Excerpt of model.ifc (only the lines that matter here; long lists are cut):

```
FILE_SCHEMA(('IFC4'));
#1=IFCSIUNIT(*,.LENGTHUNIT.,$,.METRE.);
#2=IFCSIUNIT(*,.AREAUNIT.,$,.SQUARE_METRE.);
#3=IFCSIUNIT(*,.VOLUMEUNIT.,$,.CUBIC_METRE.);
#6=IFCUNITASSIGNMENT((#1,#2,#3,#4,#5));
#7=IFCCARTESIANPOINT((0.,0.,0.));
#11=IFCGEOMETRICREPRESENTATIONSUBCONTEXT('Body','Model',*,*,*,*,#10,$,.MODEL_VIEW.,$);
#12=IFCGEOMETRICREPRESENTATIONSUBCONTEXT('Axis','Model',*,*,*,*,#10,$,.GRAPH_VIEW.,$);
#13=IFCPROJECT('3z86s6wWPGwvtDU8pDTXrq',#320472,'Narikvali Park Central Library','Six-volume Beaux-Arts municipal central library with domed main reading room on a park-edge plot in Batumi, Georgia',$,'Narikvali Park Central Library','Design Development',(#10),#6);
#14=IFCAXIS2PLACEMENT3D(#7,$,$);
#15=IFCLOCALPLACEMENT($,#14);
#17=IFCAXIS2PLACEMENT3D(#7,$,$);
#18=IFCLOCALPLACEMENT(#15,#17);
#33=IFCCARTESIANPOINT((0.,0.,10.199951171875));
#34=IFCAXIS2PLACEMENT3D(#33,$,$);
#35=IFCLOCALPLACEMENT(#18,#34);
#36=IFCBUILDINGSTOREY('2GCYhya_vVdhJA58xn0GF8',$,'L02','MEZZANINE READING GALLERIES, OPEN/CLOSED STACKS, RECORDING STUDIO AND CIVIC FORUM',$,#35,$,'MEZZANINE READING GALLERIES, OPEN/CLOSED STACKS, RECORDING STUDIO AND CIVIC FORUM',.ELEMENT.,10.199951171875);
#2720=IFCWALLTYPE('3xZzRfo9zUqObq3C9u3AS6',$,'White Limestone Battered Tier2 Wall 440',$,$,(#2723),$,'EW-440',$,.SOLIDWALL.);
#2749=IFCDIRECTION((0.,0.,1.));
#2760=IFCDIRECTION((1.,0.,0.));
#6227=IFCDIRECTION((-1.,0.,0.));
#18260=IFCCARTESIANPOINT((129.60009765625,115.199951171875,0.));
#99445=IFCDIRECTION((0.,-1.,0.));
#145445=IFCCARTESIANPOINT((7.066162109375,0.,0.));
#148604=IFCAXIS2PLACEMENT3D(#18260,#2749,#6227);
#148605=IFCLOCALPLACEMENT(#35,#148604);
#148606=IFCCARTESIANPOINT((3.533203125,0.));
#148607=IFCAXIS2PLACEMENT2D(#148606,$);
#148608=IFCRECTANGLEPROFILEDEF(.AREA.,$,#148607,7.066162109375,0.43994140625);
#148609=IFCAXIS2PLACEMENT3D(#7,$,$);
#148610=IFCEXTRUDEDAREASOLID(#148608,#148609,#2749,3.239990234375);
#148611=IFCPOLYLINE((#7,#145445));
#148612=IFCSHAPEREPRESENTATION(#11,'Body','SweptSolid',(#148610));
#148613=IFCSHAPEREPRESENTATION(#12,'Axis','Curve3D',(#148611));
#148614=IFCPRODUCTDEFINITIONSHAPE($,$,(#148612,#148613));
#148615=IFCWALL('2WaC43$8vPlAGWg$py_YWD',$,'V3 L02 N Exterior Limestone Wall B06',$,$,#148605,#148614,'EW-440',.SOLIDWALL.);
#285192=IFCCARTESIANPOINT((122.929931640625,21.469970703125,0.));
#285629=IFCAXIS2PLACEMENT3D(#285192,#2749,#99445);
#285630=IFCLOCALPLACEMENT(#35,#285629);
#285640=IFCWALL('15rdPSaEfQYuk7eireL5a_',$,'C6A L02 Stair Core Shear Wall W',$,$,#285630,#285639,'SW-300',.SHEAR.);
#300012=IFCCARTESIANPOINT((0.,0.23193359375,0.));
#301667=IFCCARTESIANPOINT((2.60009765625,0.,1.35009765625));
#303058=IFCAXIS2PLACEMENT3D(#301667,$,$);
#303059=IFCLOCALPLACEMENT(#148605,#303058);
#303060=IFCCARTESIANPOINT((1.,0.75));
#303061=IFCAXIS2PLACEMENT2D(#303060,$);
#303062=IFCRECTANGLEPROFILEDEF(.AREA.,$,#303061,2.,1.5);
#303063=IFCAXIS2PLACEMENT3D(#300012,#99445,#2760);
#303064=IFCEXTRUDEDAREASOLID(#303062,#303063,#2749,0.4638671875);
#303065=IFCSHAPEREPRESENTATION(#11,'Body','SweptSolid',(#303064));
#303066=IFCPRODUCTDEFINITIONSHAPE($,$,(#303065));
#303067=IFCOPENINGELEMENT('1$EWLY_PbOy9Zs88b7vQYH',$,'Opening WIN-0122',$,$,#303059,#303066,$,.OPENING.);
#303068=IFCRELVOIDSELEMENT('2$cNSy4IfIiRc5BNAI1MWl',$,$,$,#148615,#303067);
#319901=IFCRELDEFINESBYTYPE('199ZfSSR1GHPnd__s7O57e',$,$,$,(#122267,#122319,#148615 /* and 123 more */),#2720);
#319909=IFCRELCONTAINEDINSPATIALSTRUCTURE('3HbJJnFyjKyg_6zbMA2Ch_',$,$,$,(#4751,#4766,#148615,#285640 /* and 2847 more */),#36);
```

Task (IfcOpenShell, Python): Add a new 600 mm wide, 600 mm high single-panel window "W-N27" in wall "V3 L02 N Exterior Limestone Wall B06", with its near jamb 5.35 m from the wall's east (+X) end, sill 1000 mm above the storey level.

```python
import numpy as np
import ifcopenshell
import ifcopenshell.api.feature
import ifcopenshell.api.geometry
import ifcopenshell.api.root
import ifcopenshell.api.spatial
import ifcopenshell.geom
import ifcopenshell.util.element
import ifcopenshell.util.placement
import ifcopenshell.util.representation
import ifcopenshell.util.shape
import ifcopenshell.util.unit

model = ifcopenshell.open("model.ifc")
unit_scale = ifcopenshell.util.unit.calculate_unit_scale(model)
settings = ifcopenshell.geom.settings()


def volume(element):
    """Net volume in cubic metres, openings subtracted."""
    shape = ifcopenshell.geom.create_shape(settings, element)
    return ifcopenshell.util.shape.get_volume(shape.geometry)


wall = model.by_guid("2WaC43$8vPlAGWg$py_YWD")
storey = ifcopenshell.util.element.get_container(wall, ifc_class="IfcBuildingStorey")
context = ifcopenshell.util.representation.get_context(model, "Model", "Body", "MODEL_VIEW")
before = volume(wall)

width, height, from_end, sill = 0.6, 0.6, 5.35, 1  # metres

# The wall runs along its own X axis, and the end named is its -X end.
wall_shape = ifcopenshell.geom.create_shape(settings, wall)
x, y, z = ifcopenshell.util.shape.get_vertices(wall_shape.geometry).T
start = x.min() + from_end
face, thickness = float(y.min()), float(y.max() - y.min())
wall_matrix = ifcopenshell.util.placement.get_local_placement(wall.ObjectPlacement)
level = ifcopenshell.util.placement.get_local_placement(storey.ObjectPlacement)[2, 3]


def in_wall(x, y):
    """Placement at x, y metres in the wall's axes, at sill height."""
    matrix = wall_matrix.copy()
    matrix[:, 3] = wall_matrix @ np.array([x / unit_scale, y / unit_scale, 0.0, 1.0])
    matrix[2, 3] = level + sill / unit_scale
    return matrix


# Opening: a box that overshoots both wall faces by 50 mm.
opening = ifcopenshell.api.root.create_entity(model, ifc_class="IfcOpeningElement", predefined_type="OPENING")
box = ifcopenshell.api.geometry.add_wall_representation(
    model, context=context, length=width, height=height, thickness=thickness + 0.1
)
ifcopenshell.api.geometry.assign_representation(model, product=opening, representation=box)
ifcopenshell.api.geometry.edit_object_placement(model, product=opening, matrix=in_wall(start, face - 0.05), is_si=False)
ifcopenshell.api.feature.add_feature(model, feature=opening, element=wall)

window = ifcopenshell.api.root.create_entity(model, ifc_class="IfcWindow", name="W-N27", predefined_type="WINDOW")
window.OverallWidth, window.OverallHeight = width / unit_scale, height / unit_scale
window.PartitioningType = "SINGLE_PANEL"
body = ifcopenshell.api.geometry.add_window_representation(
    model,
    context=context,
    overall_width=window.OverallWidth,
    overall_height=window.OverallHeight,
    partition_type="SINGLE_PANEL",
)
ifcopenshell.api.geometry.assign_representation(model, product=window, representation=body)
ifcopenshell.api.spatial.assign_container(model, products=[window], relating_structure=storey)
ifcopenshell.api.feature.add_filling(model, opening=opening, element=window)

# Centre the window in the wall's thickness.
ifcopenshell.api.geometry.edit_object_placement(model, product=window, matrix=in_wall(start, face), is_si=False)
window_shape = ifcopenshell.geom.create_shape(settings, window)
depth = ifcopenshell.util.shape.get_vertices(window_shape.geometry)[:, 1]
offset = face + thickness / 2 - (depth.min() + depth.max()) / 2
ifcopenshell.api.geometry.edit_object_placement(model, product=window, matrix=in_wall(start, offset), is_si=False)

after = volume(wall)

print(f"wall volume {before:.3f} -> {after:.3f} m3")

model.write("model_edited.ifc")
```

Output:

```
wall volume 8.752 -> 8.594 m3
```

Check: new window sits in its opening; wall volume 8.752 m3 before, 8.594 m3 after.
